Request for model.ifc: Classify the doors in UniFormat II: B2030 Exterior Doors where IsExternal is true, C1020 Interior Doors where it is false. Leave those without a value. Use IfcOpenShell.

First a look at what the model holds.

```python
import ifcopenshell
import ifcopenshell.util.element

model = ifcopenshell.open("model.ifc")
print(model.schema)
print("classifications:", [c.Name for c in model.by_type("IfcClassification")])
values = [ifcopenshell.util.element.get_pset(e, "Pset_DoorCommon", "IsExternal") for e in model.by_type("IfcDoor")]
for value in (True, False, None):
    print("IsExternal", value, values.count(value))
```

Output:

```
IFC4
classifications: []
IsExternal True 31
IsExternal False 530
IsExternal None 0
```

```python
import ifcopenshell
import ifcopenshell.api.classification
import ifcopenshell.util.element

model = ifcopenshell.open("model.ifc")

system = ifcopenshell.api.classification.add_classification(model, classification="UniFormat II")

doors = model.by_type("IfcDoor")
external = {e: ifcopenshell.util.element.get_pset(e, "Pset_DoorCommon", "IsExternal") for e in doors}
for flag, code, name in ((True, "B2030", "Exterior Doors"), (False, "C1020", "Interior Doors")):
    products = [e for e in doors if external[e] is flag]
    ifcopenshell.api.classification.add_reference(
        model, products=products, classification=system, identification=code, name=name
    )
    print(code, len(products))

model.write("model_updated.ifc")
```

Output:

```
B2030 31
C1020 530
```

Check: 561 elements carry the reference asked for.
